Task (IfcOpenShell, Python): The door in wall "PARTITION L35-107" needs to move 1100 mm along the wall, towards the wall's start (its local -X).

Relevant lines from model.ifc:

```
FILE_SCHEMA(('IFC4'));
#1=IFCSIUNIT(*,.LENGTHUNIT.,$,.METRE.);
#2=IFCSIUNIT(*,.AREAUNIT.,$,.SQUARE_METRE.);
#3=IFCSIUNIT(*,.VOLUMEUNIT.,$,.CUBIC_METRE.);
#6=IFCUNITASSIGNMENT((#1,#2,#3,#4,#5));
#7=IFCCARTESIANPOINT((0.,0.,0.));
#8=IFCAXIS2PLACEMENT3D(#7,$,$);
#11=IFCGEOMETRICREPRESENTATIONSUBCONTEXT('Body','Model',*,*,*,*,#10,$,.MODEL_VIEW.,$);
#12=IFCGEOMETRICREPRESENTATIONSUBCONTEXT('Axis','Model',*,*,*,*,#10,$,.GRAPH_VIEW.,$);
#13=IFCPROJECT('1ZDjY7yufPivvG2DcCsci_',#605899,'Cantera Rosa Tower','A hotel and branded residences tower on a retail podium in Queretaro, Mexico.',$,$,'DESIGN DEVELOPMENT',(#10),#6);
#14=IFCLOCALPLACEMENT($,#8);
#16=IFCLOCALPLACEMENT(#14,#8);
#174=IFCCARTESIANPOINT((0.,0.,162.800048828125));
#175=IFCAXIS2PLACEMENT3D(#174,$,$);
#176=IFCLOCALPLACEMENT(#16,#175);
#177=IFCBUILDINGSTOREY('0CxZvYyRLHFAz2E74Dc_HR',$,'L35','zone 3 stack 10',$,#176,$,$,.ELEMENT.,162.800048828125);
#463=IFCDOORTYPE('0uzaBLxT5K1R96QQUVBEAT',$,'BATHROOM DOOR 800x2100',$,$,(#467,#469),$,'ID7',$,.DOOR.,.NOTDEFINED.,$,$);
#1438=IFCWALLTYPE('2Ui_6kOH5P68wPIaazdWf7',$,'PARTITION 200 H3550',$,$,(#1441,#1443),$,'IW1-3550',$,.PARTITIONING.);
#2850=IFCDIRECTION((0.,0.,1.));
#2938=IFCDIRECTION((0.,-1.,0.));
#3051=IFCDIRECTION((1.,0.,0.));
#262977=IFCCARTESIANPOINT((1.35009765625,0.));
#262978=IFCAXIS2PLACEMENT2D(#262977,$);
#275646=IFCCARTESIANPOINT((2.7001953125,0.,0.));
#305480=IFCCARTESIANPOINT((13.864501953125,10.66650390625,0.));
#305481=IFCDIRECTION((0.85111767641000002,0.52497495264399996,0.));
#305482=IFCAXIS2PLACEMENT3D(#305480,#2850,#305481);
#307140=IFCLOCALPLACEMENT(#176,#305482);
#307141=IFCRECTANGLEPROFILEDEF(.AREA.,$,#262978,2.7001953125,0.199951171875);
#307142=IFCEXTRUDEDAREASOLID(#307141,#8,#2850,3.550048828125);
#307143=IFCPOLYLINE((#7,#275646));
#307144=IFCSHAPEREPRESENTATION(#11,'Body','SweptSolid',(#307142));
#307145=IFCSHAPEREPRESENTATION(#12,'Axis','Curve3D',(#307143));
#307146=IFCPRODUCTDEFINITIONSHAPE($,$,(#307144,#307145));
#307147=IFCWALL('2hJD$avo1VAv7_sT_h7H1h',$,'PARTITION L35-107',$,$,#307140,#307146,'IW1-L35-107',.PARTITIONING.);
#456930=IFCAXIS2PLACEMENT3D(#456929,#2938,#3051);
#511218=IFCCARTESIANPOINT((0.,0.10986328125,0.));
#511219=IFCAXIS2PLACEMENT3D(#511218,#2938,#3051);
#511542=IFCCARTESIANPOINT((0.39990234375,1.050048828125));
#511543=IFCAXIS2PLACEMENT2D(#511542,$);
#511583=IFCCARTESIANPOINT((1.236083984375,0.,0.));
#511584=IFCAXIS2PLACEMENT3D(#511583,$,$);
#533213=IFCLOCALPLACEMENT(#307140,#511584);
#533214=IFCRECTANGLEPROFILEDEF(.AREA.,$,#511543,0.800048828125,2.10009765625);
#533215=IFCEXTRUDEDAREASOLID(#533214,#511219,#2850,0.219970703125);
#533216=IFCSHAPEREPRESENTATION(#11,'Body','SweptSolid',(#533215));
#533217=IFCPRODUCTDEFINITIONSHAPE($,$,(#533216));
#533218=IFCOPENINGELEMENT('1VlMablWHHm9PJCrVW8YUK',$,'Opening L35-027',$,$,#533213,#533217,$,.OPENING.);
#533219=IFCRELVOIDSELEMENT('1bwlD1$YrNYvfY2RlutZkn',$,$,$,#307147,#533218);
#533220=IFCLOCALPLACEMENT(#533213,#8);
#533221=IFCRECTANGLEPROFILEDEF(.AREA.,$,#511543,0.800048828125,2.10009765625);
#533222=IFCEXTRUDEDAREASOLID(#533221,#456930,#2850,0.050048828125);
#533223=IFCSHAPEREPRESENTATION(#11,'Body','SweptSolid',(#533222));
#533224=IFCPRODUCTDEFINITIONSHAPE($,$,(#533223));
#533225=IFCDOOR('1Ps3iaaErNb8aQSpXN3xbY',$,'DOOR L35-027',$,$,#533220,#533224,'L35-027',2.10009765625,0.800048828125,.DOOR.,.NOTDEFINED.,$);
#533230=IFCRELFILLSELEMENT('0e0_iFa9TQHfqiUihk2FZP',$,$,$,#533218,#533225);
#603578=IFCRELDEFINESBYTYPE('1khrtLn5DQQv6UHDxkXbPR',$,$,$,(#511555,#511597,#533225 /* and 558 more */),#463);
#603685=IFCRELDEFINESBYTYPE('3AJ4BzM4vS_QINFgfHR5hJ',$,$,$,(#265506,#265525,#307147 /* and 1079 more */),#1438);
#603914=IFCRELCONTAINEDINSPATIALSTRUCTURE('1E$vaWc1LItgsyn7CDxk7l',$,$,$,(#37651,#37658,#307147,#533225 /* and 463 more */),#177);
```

```python
import ifcopenshell
import ifcopenshell.api.geometry
import ifcopenshell.util.placement
import ifcopenshell.util.unit

model = ifcopenshell.open("model.ifc")
unit_scale = ifcopenshell.util.unit.calculate_unit_scale(model)

door = model.by_guid("1Ps3iaaErNb8aQSpXN3xbY")
opening = door.FillsVoids[0].RelatingOpeningElement
wall = opening.VoidsElements[0].RelatingBuildingElement

wall_matrix = ifcopenshell.util.placement.get_local_placement(wall.ObjectPlacement)
shift = wall_matrix[:3, 0] * -1.1 / unit_scale
before = ifcopenshell.util.placement.get_local_placement(door.ObjectPlacement)[:3, 3].copy()

# The door is placed relative to its opening, so it follows when the opening moves.
matrix = ifcopenshell.util.placement.get_local_placement(opening.ObjectPlacement)
matrix[:3, 3] += shift
ifcopenshell.api.geometry.edit_object_placement(
    model, product=opening, matrix=matrix, is_si=False, should_transform_children=True
)

after = ifcopenshell.util.placement.get_local_placement(door.ObjectPlacement)[:3, 3]
print("door moved by", (after - before).round(3) + 0.0)

model.write("model_edited.ifc")
```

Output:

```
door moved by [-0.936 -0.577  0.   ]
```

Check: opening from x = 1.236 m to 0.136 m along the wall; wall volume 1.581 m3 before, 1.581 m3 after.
